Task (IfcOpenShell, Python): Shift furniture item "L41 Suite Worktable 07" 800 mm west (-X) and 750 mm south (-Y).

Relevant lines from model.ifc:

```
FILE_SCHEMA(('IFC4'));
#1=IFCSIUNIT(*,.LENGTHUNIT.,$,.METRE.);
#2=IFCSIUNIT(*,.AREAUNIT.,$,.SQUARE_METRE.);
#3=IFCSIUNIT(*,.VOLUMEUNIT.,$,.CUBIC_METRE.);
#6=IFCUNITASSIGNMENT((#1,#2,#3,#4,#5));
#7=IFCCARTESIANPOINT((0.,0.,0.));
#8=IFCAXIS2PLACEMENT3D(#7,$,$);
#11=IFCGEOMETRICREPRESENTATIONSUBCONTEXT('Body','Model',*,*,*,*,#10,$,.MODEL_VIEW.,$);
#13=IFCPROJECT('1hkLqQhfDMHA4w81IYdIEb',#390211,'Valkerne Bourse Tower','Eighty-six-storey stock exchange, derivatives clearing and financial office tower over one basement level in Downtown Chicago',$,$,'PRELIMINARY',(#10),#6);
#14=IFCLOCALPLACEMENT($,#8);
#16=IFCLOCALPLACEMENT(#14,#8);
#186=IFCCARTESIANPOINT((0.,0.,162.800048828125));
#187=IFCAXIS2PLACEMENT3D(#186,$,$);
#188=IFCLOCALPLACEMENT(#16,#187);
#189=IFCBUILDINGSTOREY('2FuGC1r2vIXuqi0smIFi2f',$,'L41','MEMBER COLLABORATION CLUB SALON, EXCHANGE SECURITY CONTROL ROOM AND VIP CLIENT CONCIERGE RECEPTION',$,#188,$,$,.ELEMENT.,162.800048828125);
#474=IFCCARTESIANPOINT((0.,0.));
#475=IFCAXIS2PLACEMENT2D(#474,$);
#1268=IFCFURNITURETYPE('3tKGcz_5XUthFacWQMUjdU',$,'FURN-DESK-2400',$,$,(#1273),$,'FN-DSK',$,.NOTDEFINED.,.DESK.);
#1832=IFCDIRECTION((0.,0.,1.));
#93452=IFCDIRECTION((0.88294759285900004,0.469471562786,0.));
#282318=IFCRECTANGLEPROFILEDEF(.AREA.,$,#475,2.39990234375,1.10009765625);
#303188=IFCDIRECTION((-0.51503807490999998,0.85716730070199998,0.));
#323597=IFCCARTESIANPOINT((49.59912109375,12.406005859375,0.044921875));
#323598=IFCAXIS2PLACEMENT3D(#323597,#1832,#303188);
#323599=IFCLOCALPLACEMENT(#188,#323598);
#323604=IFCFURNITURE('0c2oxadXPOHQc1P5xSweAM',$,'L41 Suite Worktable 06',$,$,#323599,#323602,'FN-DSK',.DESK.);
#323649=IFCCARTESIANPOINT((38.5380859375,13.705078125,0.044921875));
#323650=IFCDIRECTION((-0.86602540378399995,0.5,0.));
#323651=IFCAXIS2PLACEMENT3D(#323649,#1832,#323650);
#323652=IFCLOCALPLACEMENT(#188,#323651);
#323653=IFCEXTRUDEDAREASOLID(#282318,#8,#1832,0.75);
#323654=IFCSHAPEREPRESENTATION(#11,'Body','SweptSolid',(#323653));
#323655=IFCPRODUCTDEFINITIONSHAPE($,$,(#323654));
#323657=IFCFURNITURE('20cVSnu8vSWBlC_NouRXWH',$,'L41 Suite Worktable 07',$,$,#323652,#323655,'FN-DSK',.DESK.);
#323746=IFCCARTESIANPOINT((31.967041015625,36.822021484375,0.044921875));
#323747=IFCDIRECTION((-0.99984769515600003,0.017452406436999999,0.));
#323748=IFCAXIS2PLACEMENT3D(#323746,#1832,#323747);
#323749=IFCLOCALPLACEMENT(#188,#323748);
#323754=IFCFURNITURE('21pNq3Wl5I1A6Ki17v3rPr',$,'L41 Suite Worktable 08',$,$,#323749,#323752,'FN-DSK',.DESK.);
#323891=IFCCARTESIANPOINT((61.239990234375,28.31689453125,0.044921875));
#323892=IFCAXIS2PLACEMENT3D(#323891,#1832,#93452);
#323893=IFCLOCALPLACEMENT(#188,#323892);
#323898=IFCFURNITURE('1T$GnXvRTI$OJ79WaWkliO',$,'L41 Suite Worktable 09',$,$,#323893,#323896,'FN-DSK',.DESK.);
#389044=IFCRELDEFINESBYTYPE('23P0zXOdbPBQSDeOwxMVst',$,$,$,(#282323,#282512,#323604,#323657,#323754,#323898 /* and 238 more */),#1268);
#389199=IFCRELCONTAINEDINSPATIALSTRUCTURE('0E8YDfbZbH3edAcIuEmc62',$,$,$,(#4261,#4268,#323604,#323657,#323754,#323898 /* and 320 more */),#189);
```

```python
import ifcopenshell
import ifcopenshell.api.geometry
import ifcopenshell.util.placement
import ifcopenshell.util.unit

model = ifcopenshell.open("model.ifc")
unit_scale = ifcopenshell.util.unit.calculate_unit_scale(model)

item = model.by_guid("20cVSnu8vSWBlC_NouRXWH")
matrix = ifcopenshell.util.placement.get_local_placement(item.ObjectPlacement)
matrix[0, 3] -= 0.8 / unit_scale
matrix[1, 3] -= 0.75 / unit_scale
ifcopenshell.api.geometry.edit_object_placement(model, product=item, matrix=matrix, is_si=False)

print(ifcopenshell.util.placement.get_local_placement(item.ObjectPlacement).round(3) + 0.0)

model.write("model_updated.ifc")
```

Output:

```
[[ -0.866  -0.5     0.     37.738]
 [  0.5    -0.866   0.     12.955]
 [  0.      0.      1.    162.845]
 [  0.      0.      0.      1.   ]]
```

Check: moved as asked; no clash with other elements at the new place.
